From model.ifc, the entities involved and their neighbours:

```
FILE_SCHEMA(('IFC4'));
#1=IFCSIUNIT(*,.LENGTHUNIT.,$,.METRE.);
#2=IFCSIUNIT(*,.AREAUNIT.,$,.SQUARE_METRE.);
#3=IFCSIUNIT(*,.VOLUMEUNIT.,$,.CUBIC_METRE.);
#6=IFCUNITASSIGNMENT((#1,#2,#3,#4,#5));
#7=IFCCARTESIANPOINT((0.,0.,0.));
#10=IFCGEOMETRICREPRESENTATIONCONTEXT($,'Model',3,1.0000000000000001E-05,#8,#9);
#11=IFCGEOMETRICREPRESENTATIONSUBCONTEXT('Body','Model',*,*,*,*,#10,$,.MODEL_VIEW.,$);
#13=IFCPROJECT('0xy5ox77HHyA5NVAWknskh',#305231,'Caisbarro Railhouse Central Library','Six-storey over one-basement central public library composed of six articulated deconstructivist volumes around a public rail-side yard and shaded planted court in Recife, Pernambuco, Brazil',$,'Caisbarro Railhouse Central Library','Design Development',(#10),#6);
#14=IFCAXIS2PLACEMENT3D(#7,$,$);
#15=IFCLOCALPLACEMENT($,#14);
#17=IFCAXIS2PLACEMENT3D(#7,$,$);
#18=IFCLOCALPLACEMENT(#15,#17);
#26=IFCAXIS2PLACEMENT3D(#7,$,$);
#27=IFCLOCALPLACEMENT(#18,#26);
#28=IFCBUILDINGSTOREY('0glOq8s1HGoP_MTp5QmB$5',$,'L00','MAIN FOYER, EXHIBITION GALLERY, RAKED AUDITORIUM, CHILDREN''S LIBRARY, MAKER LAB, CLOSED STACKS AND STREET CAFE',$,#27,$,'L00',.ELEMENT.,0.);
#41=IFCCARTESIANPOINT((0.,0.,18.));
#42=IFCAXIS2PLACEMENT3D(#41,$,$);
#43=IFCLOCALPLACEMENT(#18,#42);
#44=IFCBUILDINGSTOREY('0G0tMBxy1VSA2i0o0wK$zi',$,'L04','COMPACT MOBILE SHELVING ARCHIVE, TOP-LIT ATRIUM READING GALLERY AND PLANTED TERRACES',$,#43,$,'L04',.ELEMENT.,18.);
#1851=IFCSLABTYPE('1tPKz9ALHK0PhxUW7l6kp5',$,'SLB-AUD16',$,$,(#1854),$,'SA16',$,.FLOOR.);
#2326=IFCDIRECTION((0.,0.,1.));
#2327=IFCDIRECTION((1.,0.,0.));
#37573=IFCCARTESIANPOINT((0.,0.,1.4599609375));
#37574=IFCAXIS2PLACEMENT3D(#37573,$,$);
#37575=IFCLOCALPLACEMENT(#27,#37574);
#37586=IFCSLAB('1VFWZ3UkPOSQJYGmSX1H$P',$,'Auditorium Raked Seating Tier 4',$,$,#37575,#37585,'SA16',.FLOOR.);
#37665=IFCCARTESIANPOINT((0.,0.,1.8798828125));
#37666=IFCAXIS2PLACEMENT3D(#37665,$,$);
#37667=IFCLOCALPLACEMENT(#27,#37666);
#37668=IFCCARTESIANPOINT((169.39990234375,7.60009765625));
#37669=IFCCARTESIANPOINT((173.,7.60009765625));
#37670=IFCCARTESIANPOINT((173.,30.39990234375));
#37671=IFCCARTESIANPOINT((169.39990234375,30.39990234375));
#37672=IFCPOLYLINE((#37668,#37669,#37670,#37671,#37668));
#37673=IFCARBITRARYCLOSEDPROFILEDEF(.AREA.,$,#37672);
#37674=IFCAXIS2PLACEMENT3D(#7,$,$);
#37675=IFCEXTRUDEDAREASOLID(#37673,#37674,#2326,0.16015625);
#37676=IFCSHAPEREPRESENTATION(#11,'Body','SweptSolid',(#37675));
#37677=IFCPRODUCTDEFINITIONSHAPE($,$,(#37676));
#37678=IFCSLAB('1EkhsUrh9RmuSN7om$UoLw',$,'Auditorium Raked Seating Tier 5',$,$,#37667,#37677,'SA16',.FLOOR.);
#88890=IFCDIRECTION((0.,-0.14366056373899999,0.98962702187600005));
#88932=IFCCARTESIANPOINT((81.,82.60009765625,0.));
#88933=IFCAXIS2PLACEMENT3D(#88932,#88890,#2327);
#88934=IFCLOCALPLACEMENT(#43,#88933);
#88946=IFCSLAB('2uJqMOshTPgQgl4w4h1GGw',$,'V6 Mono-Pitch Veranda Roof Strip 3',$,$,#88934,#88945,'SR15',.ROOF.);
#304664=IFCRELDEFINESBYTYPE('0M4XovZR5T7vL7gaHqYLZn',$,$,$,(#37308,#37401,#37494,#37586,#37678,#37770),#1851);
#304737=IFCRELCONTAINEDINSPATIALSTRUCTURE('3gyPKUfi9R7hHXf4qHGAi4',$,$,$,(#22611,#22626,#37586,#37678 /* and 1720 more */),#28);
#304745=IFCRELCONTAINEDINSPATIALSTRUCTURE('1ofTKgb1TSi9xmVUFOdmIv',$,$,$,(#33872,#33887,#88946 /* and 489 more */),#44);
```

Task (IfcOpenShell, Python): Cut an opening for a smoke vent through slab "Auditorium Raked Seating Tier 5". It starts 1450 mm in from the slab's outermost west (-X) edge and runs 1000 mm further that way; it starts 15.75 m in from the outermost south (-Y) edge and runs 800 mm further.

```python
import numpy as np
import ifcopenshell
import ifcopenshell.api.feature
import ifcopenshell.api.geometry
import ifcopenshell.api.root
import ifcopenshell.geom
import ifcopenshell.util.placement
import ifcopenshell.util.representation
import ifcopenshell.util.shape
import ifcopenshell.util.unit

model = ifcopenshell.open("model.ifc")
unit_scale = ifcopenshell.util.unit.calculate_unit_scale(model)
settings = ifcopenshell.geom.settings()


def volume(element):
    """Net volume in cubic metres, openings subtracted."""
    shape = ifcopenshell.geom.create_shape(settings, element)
    return ifcopenshell.util.shape.get_volume(shape.geometry)


slab = model.by_id(37678)
before = volume(slab)

# Extent in the slab's own axes, in metres. The edges named are its -X and -Y sides.
slab_shape = ifcopenshell.geom.create_shape(settings, slab)
vertices = ifcopenshell.util.shape.get_vertices(slab_shape.geometry)
x_min, y_min, bottom = vertices.min(axis=0)
top = vertices[:, 2].max()

opening = ifcopenshell.api.root.create_entity(model, ifc_class="IfcOpeningElement", name="Smoke vent opening", predefined_type="OPENING")
context = ifcopenshell.util.representation.get_context(model, "Model", "Body", "MODEL_VIEW")
width, depth = 1, 0.8
outline = [(0.0, 0.0), (width, 0.0), (width, depth), (0.0, depth), (0.0, 0.0)]
# Overshoot both faces by 50 mm so the cut is clean.
shape = ifcopenshell.api.geometry.add_slab_representation(
    model, context=context, depth=top - bottom + 0.1, polyline=outline
)
ifcopenshell.api.geometry.assign_representation(model, product=opening, representation=shape)

matrix = ifcopenshell.util.placement.get_local_placement(slab.ObjectPlacement)
matrix[:, 3] = matrix @ np.append(np.array([x_min + 1.45, y_min + 15.75, bottom - 0.05]) / unit_scale, 1.0)
ifcopenshell.api.geometry.edit_object_placement(model, product=opening, matrix=matrix, is_si=False)
ifcopenshell.api.feature.add_feature(model, feature=opening, element=slab)

after = volume(slab)

print(f"slab volume {before:.3f} -> {after:.3f} m3")

model.write("model_updated.ifc")
```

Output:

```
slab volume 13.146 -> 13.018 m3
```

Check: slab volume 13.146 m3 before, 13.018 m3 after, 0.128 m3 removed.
